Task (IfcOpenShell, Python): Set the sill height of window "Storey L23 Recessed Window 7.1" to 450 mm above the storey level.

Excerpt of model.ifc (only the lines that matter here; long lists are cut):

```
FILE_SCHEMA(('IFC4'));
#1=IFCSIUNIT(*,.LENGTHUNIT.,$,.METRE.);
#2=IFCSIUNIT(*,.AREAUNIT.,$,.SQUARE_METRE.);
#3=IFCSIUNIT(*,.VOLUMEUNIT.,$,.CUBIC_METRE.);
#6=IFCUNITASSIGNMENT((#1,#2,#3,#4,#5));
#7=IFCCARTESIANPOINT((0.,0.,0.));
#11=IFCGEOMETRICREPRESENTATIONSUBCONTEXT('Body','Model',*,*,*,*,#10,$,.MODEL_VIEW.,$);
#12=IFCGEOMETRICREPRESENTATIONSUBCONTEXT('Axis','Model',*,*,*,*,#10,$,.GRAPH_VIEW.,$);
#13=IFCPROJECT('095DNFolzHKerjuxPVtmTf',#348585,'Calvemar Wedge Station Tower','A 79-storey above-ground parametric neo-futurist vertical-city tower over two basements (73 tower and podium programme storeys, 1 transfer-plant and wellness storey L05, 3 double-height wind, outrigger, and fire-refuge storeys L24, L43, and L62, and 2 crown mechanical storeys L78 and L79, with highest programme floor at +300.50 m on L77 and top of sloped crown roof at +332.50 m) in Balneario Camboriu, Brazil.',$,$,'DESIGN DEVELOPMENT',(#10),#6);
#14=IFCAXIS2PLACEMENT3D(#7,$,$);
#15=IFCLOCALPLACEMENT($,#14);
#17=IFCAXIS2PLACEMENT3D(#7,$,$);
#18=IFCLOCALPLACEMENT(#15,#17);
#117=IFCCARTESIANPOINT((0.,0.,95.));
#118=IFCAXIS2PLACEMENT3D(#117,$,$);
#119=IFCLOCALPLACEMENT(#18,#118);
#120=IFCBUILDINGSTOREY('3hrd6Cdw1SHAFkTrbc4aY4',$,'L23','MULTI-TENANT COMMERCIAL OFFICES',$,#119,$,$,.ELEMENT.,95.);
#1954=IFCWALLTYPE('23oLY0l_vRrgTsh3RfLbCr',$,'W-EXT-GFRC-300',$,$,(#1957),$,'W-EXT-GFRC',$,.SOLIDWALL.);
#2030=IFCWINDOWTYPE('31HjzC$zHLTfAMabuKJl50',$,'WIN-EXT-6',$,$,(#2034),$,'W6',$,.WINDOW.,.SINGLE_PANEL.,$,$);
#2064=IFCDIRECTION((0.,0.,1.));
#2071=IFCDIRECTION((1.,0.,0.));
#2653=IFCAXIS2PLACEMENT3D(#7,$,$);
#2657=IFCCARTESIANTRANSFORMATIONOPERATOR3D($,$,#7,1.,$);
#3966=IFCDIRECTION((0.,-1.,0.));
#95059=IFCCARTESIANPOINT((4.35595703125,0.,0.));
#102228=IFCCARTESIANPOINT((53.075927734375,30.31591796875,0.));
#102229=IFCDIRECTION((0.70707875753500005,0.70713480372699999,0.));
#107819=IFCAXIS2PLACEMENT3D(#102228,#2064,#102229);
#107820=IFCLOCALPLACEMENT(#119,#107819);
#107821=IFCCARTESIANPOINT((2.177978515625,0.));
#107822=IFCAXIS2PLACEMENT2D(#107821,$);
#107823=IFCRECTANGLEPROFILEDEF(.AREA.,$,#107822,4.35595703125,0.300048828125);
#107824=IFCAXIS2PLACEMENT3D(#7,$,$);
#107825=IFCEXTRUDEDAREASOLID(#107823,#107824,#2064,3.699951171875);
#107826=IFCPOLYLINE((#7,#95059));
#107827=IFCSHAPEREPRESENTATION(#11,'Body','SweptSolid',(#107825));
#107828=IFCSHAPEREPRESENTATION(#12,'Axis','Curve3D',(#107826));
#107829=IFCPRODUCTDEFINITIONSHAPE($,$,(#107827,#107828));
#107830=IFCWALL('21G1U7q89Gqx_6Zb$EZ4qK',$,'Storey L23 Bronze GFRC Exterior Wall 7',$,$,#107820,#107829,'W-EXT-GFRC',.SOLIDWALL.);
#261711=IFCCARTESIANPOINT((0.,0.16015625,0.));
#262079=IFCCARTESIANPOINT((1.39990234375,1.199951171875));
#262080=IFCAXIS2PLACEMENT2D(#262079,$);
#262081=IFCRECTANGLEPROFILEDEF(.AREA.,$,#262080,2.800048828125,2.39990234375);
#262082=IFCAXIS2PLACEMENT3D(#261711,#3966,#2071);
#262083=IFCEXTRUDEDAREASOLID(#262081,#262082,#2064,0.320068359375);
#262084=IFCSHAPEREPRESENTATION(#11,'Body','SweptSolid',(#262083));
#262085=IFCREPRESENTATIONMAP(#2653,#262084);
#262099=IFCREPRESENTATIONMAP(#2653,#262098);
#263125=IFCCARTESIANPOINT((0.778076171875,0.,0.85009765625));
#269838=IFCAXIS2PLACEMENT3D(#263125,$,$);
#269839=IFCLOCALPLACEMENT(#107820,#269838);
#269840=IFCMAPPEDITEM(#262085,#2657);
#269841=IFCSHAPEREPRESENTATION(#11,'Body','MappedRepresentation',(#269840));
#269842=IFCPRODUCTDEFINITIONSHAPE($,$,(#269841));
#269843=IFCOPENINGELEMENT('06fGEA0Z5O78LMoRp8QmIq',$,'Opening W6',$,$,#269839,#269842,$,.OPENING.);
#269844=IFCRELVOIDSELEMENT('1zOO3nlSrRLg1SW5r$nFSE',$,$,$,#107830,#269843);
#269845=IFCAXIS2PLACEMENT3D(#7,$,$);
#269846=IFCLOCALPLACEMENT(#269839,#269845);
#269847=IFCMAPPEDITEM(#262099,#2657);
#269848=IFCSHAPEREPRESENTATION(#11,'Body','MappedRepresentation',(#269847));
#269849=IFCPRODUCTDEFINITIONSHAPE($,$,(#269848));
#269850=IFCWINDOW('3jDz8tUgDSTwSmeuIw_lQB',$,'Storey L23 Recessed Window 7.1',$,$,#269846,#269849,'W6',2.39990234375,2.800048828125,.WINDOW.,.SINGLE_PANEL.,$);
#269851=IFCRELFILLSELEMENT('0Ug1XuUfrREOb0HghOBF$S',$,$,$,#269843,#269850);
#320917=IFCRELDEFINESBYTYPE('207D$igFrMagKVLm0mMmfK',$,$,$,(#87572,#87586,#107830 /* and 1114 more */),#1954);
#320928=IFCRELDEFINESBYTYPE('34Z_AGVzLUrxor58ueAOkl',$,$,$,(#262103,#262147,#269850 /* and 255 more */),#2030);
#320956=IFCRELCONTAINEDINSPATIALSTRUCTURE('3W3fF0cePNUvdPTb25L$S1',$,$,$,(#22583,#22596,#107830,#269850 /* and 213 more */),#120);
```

```python
import numpy as np
import ifcopenshell
import ifcopenshell.api.geometry
import ifcopenshell.geom
import ifcopenshell.util.element
import ifcopenshell.util.placement
import ifcopenshell.util.shape
import ifcopenshell.util.unit

model = ifcopenshell.open("model.ifc")
unit_scale = ifcopenshell.util.unit.calculate_unit_scale(model)

window = model.by_id(269850)
opening = window.FillsVoids[0].RelatingOpeningElement
storey = ifcopenshell.util.element.get_container(window, ifc_class="IfcBuildingStorey")
level = ifcopenshell.util.placement.get_local_placement(storey.ObjectPlacement)[2, 3]

# The opening's origin need not be at the sill, so measure its lowest point.
shape = ifcopenshell.geom.create_shape(ifcopenshell.geom.settings(), opening)
bottom = ifcopenshell.util.shape.get_shape_bottom_elevation(shape, shape.geometry) / unit_scale
dz = level + 0.45 - bottom

shift = np.array([0.0, 0.0, dz])
# The window is placed relative to its opening, so it follows when the opening moves.
matrix = ifcopenshell.util.placement.get_local_placement(opening.ObjectPlacement)
matrix[:3, 3] += shift
ifcopenshell.api.geometry.edit_object_placement(
    model, product=opening, matrix=matrix, is_si=False, should_transform_children=True
)

print(f"moved by {dz * unit_scale:+.3f} m")

model.write("model-out.ifc")
```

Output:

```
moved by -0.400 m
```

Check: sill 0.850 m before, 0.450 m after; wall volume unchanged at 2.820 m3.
